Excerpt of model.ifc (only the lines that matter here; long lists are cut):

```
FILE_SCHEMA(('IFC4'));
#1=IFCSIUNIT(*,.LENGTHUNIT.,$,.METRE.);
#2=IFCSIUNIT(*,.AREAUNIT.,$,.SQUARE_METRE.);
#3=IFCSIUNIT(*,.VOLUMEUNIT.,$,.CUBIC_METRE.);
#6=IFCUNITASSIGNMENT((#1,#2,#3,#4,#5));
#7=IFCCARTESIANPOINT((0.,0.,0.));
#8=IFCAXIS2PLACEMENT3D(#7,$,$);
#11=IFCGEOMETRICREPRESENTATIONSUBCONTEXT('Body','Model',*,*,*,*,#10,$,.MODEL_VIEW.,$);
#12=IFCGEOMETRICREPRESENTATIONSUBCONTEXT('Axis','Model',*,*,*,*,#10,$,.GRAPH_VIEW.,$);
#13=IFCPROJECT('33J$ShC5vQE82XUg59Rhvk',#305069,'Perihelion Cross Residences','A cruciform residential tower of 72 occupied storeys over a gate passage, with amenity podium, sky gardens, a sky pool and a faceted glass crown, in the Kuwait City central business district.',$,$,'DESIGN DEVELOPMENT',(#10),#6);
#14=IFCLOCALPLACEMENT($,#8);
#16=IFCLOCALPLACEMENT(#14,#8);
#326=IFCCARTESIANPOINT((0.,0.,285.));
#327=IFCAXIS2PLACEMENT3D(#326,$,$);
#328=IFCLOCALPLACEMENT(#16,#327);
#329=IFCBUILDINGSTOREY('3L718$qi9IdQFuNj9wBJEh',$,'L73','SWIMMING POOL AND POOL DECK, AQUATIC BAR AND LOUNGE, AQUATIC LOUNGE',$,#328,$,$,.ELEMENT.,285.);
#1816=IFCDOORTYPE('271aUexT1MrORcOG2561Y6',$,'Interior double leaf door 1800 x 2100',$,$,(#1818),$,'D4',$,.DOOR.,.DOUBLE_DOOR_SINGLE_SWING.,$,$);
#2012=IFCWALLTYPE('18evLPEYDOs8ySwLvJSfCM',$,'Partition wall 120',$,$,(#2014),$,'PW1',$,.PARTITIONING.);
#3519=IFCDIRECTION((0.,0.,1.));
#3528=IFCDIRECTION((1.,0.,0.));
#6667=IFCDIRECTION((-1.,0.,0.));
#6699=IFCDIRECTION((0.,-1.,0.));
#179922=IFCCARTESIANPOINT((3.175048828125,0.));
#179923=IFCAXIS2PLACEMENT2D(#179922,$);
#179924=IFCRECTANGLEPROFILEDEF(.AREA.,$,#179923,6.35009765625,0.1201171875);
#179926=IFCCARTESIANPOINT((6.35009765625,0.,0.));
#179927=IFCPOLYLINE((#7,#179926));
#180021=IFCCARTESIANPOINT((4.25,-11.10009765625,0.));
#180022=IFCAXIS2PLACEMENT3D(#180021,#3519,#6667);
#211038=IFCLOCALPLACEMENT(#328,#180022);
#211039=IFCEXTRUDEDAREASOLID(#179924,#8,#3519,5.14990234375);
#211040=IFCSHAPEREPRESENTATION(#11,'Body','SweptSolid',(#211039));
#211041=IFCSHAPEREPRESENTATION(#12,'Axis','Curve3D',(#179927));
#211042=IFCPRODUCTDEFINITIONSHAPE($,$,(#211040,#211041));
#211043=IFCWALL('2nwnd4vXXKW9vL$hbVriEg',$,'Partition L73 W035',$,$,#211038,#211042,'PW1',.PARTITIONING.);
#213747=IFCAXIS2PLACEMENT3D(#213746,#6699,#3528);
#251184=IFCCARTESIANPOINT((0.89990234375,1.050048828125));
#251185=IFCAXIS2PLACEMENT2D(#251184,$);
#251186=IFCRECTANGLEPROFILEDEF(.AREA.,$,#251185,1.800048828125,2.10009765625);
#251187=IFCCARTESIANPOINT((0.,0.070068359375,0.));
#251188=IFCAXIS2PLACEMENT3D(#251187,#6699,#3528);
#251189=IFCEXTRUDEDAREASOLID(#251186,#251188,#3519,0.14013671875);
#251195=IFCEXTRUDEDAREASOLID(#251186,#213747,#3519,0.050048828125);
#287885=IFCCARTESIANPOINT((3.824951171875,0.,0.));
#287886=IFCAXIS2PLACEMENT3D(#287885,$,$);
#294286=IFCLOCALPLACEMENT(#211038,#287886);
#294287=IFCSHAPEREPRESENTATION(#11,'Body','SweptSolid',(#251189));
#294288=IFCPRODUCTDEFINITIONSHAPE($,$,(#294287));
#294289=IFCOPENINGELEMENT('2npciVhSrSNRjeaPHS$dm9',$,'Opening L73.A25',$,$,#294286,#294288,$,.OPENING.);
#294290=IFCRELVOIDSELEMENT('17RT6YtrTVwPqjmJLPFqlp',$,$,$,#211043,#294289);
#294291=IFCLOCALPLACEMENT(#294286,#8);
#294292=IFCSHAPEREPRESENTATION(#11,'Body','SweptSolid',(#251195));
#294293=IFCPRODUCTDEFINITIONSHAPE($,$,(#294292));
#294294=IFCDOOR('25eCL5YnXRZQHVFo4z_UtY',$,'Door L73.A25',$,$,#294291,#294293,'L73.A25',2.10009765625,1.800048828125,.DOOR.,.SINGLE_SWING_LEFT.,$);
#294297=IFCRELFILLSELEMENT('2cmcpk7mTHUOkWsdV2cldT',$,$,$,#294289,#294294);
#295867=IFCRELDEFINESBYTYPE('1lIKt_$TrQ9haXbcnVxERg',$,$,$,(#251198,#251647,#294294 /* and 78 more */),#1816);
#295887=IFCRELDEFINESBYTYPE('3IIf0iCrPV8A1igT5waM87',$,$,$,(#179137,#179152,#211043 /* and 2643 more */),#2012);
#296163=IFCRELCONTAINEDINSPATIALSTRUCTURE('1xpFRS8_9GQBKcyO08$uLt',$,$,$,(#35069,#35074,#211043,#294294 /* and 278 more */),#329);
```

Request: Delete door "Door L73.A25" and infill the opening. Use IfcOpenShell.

```python
import ifcopenshell
import ifcopenshell.api.feature
import ifcopenshell.api.root
import ifcopenshell.geom
import ifcopenshell.util.shape

model = ifcopenshell.open("model.ifc")
settings = ifcopenshell.geom.settings()


def volume(element):
    """Net volume in cubic metres, openings subtracted."""
    shape = ifcopenshell.geom.create_shape(settings, element)
    return ifcopenshell.util.shape.get_volume(shape.geometry)


door = model.by_guid("25eCL5YnXRZQHVFo4z_UtY")
opening = door.FillsVoids[0].RelatingOpeningElement
wall = opening.VoidsElements[0].RelatingBuildingElement
before = volume(wall)

ifcopenshell.api.root.remove_product(model, product=door)
ifcopenshell.api.feature.remove_feature(model, feature=opening)

after = volume(wall)

print(f"wall volume {before:.3f} -> {after:.3f} m3")

model.write("model-out.ifc")
```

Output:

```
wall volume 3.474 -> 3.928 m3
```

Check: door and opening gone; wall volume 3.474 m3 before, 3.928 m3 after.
